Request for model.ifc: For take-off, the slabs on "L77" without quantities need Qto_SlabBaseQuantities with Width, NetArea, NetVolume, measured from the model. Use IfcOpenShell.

First a look at what the model holds.

```python
import ifcopenshell
import ifcopenshell.util.element
import ifcopenshell.util.unit

model = ifcopenshell.open("model.ifc")
print(model.schema)
for unit_type in ("LENGTHUNIT", "AREAUNIT", "VOLUMEUNIT"):
    print(unit_type, ifcopenshell.util.unit.calculate_unit_scale(model, unit_type))
storey = next(s for s in model.by_type("IfcBuildingStorey") if s.Name == "L77")
slabs = [e for e in ifcopenshell.util.element.get_decomposition(storey) if e.is_a("IfcSlab")]
for e in sorted(slabs, key=lambda e: e.id()):
    print(e.id(), e.is_a(), e.Name, list(ifcopenshell.util.element.get_psets(e, qtos_only=True)), sep=" | ")
```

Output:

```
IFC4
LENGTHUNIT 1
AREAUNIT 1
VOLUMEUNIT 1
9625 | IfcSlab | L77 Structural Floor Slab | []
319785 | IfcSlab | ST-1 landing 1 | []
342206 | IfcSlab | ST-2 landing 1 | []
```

```python
import ifcopenshell
import ifcopenshell.api.pset
import ifcopenshell.geom
import ifcopenshell.util.element
import ifcopenshell.util.shape
import ifcopenshell.util.unit

model = ifcopenshell.open("model.ifc")
unit_scale = ifcopenshell.util.unit.calculate_unit_scale(model)
area_scale = ifcopenshell.util.unit.calculate_unit_scale(model, "AREAUNIT")
volume_scale = ifcopenshell.util.unit.calculate_unit_scale(model, "VOLUMEUNIT")
settings = ifcopenshell.geom.settings()

storey = next(s for s in model.by_type("IfcBuildingStorey") if s.Name == "L77")
slabs = [e for e in ifcopenshell.util.element.get_decomposition(storey) if e.is_a("IfcSlab")]

for e in sorted(slabs, key=lambda e: e.id()):
    if ifcopenshell.util.element.get_psets(e, qtos_only=True, should_inherit=False):
        continue
    # Geometry comes back in metres, in the element's own axes.
    shape = ifcopenshell.geom.create_shape(settings, e)
    values = {
        "Width": ifcopenshell.util.shape.get_z(shape.geometry) / unit_scale,
        "NetArea": ifcopenshell.util.shape.get_footprint_area(shape.geometry) / area_scale,
        "NetVolume": ifcopenshell.util.shape.get_volume(shape.geometry) / volume_scale,
    }
    qto = ifcopenshell.api.pset.add_qto(model, product=e, name="Qto_SlabBaseQuantities")
    ifcopenshell.api.pset.edit_qto(model, qto=qto, properties=values)
    print(e.id(), {k: round(v, 3) for k, v in values.items()})

model.write("model_edited.ifc")
```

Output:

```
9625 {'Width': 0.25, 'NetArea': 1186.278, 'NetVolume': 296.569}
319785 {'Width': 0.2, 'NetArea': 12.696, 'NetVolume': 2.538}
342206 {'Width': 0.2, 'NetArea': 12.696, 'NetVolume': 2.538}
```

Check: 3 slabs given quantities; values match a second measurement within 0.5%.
